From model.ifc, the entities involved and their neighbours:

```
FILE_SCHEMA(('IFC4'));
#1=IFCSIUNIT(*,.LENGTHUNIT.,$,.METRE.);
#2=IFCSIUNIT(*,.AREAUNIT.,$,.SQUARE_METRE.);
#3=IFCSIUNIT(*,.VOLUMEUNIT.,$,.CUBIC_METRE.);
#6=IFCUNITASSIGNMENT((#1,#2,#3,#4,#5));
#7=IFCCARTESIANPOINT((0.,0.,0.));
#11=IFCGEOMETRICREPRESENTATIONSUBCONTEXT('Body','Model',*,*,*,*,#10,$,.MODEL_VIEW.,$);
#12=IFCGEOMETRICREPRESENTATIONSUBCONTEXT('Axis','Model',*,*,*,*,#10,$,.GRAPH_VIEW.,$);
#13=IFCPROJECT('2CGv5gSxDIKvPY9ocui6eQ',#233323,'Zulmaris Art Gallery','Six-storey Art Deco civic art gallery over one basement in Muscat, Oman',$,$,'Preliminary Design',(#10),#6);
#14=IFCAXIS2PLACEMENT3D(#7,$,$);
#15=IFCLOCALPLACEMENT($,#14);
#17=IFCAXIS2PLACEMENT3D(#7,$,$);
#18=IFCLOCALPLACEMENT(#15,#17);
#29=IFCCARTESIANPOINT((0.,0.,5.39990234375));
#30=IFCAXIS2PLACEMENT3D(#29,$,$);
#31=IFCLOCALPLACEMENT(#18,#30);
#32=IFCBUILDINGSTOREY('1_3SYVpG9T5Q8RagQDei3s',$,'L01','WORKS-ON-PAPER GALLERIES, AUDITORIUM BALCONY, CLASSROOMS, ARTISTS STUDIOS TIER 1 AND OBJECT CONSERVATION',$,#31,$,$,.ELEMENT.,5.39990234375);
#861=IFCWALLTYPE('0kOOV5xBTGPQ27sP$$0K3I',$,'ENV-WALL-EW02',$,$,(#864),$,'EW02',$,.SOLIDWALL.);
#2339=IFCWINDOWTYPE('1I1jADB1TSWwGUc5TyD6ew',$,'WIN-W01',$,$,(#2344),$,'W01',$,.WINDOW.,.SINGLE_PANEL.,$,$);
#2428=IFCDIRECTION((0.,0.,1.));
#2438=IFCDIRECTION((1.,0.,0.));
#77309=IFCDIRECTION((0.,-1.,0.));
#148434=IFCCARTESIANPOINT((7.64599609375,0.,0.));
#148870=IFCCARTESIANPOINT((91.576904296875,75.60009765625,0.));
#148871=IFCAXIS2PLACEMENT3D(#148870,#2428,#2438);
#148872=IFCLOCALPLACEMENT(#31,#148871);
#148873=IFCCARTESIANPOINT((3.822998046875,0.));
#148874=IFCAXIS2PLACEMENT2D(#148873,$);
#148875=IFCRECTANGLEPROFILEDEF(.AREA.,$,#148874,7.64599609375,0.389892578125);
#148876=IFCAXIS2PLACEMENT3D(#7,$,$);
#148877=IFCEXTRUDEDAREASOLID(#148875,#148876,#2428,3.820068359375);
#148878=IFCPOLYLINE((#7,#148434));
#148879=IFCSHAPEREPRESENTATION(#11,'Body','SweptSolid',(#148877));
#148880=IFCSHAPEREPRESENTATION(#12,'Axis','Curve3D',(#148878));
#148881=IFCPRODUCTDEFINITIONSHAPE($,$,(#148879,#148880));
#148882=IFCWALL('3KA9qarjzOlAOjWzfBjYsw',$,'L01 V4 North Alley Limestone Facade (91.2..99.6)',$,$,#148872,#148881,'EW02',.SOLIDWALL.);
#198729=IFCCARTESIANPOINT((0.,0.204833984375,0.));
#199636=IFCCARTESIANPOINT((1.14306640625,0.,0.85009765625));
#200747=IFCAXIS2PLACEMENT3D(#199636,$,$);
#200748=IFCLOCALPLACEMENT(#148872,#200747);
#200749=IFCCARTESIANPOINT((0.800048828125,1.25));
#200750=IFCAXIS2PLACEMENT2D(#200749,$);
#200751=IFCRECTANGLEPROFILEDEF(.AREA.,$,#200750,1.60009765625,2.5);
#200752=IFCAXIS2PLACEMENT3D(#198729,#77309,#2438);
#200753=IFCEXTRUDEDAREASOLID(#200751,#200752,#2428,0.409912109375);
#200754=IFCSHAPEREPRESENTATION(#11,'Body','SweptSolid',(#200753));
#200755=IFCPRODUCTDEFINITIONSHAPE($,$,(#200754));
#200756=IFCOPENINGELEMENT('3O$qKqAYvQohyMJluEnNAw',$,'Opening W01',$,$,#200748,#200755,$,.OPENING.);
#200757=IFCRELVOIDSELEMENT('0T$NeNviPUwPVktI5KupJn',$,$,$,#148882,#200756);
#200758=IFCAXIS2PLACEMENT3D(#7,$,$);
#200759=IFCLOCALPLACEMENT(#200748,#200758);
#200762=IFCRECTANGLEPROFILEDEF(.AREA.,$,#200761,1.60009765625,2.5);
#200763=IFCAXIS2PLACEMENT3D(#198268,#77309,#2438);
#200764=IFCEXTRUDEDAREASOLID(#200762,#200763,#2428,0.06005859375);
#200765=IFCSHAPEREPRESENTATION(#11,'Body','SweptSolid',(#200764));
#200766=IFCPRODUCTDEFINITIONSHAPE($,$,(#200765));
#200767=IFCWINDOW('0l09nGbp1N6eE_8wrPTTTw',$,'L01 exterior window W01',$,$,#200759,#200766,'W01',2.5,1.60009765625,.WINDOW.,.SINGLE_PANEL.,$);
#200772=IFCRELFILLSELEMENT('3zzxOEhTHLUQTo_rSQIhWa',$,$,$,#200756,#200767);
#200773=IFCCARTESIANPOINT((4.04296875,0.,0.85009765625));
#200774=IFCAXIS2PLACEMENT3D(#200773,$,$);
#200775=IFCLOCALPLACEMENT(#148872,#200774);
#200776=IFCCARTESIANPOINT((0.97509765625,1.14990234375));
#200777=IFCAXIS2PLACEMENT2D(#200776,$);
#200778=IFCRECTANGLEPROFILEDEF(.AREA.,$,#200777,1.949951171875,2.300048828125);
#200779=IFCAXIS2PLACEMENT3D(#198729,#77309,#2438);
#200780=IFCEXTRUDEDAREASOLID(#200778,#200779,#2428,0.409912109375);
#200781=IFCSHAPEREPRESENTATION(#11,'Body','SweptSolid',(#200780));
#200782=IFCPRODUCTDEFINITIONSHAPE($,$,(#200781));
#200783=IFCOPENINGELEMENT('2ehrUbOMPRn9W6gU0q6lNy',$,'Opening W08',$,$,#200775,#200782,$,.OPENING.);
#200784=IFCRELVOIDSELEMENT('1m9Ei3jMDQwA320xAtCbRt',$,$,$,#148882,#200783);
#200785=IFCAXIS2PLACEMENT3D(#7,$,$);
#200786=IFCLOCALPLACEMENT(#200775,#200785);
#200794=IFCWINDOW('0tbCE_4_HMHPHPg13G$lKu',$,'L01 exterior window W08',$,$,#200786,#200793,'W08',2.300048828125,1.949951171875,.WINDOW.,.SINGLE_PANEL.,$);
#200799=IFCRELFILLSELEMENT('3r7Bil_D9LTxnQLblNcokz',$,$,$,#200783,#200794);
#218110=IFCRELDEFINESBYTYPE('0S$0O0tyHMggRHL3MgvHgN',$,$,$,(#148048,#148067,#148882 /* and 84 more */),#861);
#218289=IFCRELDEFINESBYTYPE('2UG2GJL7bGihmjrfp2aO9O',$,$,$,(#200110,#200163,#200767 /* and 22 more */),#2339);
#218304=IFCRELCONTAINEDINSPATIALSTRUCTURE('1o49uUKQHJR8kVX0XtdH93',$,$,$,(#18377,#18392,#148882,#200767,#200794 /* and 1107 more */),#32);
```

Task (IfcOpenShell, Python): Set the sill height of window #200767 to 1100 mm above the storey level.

```python
import numpy as np
import ifcopenshell
import ifcopenshell.api.geometry
import ifcopenshell.geom
import ifcopenshell.util.element
import ifcopenshell.util.placement
import ifcopenshell.util.shape
import ifcopenshell.util.unit

model = ifcopenshell.open("model.ifc")
unit_scale = ifcopenshell.util.unit.calculate_unit_scale(model)

window = model.by_guid("0l09nGbp1N6eE_8wrPTTTw")
opening = window.FillsVoids[0].RelatingOpeningElement
storey = ifcopenshell.util.element.get_container(window, ifc_class="IfcBuildingStorey")
level = ifcopenshell.util.placement.get_local_placement(storey.ObjectPlacement)[2, 3]

# The opening's origin need not be at the sill, so measure its lowest point.
shape = ifcopenshell.geom.create_shape(ifcopenshell.geom.settings(), opening)
bottom = ifcopenshell.util.shape.get_shape_bottom_elevation(shape, shape.geometry) / unit_scale
dz = level + 1.1 - bottom

shift = np.array([0.0, 0.0, dz])
# The window is placed relative to its opening, so it follows when the opening moves.
matrix = ifcopenshell.util.placement.get_local_placement(opening.ObjectPlacement)
matrix[:3, 3] += shift
ifcopenshell.api.geometry.edit_object_placement(
    model, product=opening, matrix=matrix, is_si=False, should_transform_children=True
)

print(f"moved by {dz * unit_scale:+.3f} m")

model.write("model_edited.ifc")
```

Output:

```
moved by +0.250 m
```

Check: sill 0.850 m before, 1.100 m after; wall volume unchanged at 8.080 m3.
